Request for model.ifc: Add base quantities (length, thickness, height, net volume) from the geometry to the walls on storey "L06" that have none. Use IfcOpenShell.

First a look at what the model holds.

```python
import ifcopenshell
import ifcopenshell.util.element
import ifcopenshell.util.unit

model = ifcopenshell.open("model.ifc")
print(model.schema)
for unit_type in ("LENGTHUNIT", "AREAUNIT", "VOLUMEUNIT"):
    print(unit_type, ifcopenshell.util.unit.calculate_unit_scale(model, unit_type))
storey = next(s for s in model.by_type("IfcBuildingStorey") if s.Name == "L06")
walls = [e for e in ifcopenshell.util.element.get_decomposition(storey) if e.is_a("IfcWall")]
for e in sorted(walls, key=lambda e: e.id()):
    print(e.id(), e.is_a(), e.Name, list(ifcopenshell.util.element.get_psets(e, qtos_only=True)), sep=" | ")
```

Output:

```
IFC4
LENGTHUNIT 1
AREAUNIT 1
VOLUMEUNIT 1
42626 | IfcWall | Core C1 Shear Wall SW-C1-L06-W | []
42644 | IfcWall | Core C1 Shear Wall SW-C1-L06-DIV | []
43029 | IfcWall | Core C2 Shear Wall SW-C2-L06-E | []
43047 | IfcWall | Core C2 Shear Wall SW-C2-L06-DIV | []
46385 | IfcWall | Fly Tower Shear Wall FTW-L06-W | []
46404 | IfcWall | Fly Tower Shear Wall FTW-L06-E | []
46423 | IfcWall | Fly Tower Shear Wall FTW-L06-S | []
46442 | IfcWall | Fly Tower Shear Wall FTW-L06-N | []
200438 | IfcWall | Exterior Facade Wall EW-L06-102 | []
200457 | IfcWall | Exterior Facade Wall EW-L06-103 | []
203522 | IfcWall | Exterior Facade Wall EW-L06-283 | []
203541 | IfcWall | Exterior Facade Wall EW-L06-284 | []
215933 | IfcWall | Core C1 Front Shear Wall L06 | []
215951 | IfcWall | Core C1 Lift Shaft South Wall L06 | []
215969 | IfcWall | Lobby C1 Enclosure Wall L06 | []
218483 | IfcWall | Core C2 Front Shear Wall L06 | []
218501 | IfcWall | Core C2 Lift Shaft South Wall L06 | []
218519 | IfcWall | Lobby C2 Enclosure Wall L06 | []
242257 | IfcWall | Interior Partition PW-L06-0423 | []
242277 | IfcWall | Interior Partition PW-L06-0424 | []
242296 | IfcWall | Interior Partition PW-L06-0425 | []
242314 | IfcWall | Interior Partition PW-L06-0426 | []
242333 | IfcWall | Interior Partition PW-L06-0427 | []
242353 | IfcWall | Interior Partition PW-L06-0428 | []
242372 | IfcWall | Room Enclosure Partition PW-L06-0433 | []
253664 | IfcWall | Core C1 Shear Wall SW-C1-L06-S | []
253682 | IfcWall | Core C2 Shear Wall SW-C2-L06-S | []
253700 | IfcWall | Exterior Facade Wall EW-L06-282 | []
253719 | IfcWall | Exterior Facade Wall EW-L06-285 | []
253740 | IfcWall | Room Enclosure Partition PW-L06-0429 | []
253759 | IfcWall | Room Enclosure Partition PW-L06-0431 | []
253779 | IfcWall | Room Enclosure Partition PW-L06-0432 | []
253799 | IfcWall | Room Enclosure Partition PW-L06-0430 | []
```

```python
import ifcopenshell
import ifcopenshell.api.pset
import ifcopenshell.geom
import ifcopenshell.util.element
import ifcopenshell.util.shape
import ifcopenshell.util.unit

model = ifcopenshell.open("model.ifc")
unit_scale = ifcopenshell.util.unit.calculate_unit_scale(model)
volume_scale = ifcopenshell.util.unit.calculate_unit_scale(model, "VOLUMEUNIT")
settings = ifcopenshell.geom.settings()

storey = next(s for s in model.by_type("IfcBuildingStorey") if s.Name == "L06")
walls = [e for e in ifcopenshell.util.element.get_decomposition(storey) if e.is_a("IfcWall")]

for e in sorted(walls, key=lambda e: e.id()):
    if ifcopenshell.util.element.get_psets(e, qtos_only=True, should_inherit=False):
        continue
    # Geometry comes back in metres, in the element's own axes.
    shape = ifcopenshell.geom.create_shape(settings, e)
    values = {
        "Length": ifcopenshell.util.shape.get_x(shape.geometry) / unit_scale,
        "Width": ifcopenshell.util.shape.get_y(shape.geometry) / unit_scale,
        "Height": ifcopenshell.util.shape.get_z(shape.geometry) / unit_scale,
        "NetVolume": ifcopenshell.util.shape.get_volume(shape.geometry) / volume_scale,
    }
    qto = ifcopenshell.api.pset.add_qto(model, product=e, name="Qto_WallBaseQuantities")
    ifcopenshell.api.pset.edit_qto(model, qto=qto, properties=values)
    print(e.id(), {k: round(v, 3) for k, v in values.items()})

model.write("model-out.ifc")
```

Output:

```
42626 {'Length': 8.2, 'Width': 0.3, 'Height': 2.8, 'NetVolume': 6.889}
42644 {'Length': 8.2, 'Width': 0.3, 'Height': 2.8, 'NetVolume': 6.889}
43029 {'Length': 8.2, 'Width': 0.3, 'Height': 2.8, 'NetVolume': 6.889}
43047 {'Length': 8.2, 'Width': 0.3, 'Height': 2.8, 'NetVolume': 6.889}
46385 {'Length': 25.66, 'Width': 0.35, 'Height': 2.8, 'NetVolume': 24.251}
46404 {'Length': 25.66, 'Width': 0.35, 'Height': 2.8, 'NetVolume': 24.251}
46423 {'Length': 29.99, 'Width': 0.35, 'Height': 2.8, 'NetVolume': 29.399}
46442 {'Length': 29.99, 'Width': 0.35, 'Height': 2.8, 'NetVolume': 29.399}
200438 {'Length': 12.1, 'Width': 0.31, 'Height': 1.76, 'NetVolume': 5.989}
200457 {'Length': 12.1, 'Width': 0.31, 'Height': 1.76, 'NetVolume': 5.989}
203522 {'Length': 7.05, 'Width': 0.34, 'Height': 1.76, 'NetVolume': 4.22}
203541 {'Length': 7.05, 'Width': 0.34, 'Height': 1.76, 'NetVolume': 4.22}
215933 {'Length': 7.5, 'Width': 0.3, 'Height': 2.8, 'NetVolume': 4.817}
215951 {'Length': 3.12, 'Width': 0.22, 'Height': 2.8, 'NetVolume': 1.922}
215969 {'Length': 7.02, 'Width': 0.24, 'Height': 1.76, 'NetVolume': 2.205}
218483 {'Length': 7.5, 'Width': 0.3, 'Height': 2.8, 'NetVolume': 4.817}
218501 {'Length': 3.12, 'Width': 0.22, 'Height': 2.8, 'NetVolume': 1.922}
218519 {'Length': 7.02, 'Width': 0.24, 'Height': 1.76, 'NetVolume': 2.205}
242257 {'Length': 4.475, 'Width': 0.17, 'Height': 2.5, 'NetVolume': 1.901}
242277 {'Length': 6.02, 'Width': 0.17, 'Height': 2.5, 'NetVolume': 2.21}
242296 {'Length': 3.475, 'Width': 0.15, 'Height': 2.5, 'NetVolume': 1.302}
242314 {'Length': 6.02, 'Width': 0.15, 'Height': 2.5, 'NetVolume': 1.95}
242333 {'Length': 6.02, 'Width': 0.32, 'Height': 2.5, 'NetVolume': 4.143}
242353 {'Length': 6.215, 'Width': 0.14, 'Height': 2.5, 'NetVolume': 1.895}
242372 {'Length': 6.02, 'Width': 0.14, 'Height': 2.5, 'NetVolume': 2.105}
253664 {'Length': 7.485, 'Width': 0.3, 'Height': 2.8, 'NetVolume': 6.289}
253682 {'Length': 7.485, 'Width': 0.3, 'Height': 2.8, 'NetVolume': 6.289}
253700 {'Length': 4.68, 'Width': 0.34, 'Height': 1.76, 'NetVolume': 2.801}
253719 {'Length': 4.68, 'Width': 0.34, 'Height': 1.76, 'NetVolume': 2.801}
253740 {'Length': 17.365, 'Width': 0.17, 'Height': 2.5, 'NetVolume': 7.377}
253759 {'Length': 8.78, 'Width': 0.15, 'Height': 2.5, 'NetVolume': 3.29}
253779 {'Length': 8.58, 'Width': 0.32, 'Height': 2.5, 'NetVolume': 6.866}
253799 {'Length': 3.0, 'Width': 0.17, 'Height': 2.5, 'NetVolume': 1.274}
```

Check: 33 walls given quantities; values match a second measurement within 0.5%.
